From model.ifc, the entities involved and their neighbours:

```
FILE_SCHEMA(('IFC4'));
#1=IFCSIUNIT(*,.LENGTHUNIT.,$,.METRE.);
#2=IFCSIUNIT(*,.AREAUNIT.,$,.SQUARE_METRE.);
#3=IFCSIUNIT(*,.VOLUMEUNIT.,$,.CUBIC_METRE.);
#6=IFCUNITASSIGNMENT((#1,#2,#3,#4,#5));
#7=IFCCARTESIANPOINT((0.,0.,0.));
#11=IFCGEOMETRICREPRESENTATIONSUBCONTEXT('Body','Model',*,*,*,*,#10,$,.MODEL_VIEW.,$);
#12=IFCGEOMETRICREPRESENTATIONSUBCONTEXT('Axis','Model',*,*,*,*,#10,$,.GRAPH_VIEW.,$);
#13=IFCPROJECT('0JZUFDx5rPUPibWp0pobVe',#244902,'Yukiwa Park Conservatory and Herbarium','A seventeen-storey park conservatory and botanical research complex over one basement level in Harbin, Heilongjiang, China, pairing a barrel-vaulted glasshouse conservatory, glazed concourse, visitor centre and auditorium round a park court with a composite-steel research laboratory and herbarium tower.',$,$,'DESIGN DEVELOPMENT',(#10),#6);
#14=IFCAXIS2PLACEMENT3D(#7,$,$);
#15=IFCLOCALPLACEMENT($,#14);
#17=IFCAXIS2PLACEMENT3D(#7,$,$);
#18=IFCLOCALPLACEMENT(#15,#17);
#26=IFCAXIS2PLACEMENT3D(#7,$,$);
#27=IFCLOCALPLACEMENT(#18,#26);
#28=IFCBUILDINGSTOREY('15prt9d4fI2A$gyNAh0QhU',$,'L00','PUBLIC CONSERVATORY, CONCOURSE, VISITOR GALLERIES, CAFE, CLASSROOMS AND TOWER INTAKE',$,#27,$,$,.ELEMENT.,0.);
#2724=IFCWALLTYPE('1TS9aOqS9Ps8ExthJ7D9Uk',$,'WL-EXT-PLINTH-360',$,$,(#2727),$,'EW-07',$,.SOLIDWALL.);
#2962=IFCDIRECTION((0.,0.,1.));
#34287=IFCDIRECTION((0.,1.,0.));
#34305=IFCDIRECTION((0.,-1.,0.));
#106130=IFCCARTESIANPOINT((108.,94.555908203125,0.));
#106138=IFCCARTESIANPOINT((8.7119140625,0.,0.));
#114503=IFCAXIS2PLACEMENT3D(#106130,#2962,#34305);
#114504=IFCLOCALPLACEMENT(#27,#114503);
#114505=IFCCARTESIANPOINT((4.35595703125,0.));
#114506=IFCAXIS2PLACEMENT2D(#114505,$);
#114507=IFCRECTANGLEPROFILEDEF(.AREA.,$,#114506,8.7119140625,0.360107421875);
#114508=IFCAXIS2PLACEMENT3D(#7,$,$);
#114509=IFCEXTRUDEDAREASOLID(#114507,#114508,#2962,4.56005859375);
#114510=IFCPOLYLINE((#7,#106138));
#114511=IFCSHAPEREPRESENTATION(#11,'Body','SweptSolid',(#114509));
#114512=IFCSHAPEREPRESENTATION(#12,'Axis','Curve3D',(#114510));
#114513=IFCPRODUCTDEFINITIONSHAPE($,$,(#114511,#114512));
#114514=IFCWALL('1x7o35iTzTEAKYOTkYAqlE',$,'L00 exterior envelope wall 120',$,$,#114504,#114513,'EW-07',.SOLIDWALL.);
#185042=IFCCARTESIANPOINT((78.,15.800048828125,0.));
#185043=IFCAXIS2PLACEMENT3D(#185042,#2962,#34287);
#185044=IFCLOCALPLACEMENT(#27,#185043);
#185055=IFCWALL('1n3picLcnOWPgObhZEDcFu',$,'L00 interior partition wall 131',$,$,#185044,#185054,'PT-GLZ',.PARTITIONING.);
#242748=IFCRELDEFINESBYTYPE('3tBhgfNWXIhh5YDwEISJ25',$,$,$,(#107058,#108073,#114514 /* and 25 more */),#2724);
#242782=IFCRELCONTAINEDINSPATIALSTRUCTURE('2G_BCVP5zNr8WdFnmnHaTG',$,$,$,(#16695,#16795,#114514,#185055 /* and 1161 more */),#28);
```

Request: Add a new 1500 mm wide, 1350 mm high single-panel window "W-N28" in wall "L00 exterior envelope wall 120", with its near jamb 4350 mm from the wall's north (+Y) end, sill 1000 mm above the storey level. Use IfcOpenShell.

```python
import numpy as np
import ifcopenshell
import ifcopenshell.api.feature
import ifcopenshell.api.geometry
import ifcopenshell.api.root
import ifcopenshell.api.spatial
import ifcopenshell.geom
import ifcopenshell.util.element
import ifcopenshell.util.placement
import ifcopenshell.util.representation
import ifcopenshell.util.shape
import ifcopenshell.util.unit

model = ifcopenshell.open("model.ifc")
unit_scale = ifcopenshell.util.unit.calculate_unit_scale(model)
settings = ifcopenshell.geom.settings()


def volume(element):
    """Net volume in cubic metres, openings subtracted."""
    shape = ifcopenshell.geom.create_shape(settings, element)
    return ifcopenshell.util.shape.get_volume(shape.geometry)


wall = model.by_guid("1x7o35iTzTEAKYOTkYAqlE")
storey = ifcopenshell.util.element.get_container(wall, ifc_class="IfcBuildingStorey")
context = ifcopenshell.util.representation.get_context(model, "Model", "Body", "MODEL_VIEW")
before = volume(wall)

width, height, from_end, sill = 1.5, 1.35, 4.35, 1  # metres

# The wall runs along its own X axis, and the end named is its -X end.
wall_shape = ifcopenshell.geom.create_shape(settings, wall)
x, y, z = ifcopenshell.util.shape.get_vertices(wall_shape.geometry).T
start = x.min() + from_end
face, thickness = float(y.min()), float(y.max() - y.min())
wall_matrix = ifcopenshell.util.placement.get_local_placement(wall.ObjectPlacement)
level = ifcopenshell.util.placement.get_local_placement(storey.ObjectPlacement)[2, 3]


def in_wall(x, y):
    """Placement at x, y metres in the wall's axes, at sill height."""
    matrix = wall_matrix.copy()
    matrix[:, 3] = wall_matrix @ np.array([x / unit_scale, y / unit_scale, 0.0, 1.0])
    matrix[2, 3] = level + sill / unit_scale
    return matrix


# Opening: a box that overshoots both wall faces by 50 mm.
opening = ifcopenshell.api.root.create_entity(model, ifc_class="IfcOpeningElement", predefined_type="OPENING")
box = ifcopenshell.api.geometry.add_wall_representation(
    model, context=context, length=width, height=height, thickness=thickness + 0.1
)
ifcopenshell.api.geometry.assign_representation(model, product=opening, representation=box)
ifcopenshell.api.geometry.edit_object_placement(model, product=opening, matrix=in_wall(start, face - 0.05), is_si=False)
ifcopenshell.api.feature.add_feature(model, feature=opening, element=wall)

window = ifcopenshell.api.root.create_entity(model, ifc_class="IfcWindow", name="W-N28", predefined_type="WINDOW")
window.OverallWidth, window.OverallHeight = width / unit_scale, height / unit_scale
window.PartitioningType = "SINGLE_PANEL"
body = ifcopenshell.api.geometry.add_window_representation(
    model,
    context=context,
    overall_width=window.OverallWidth,
    overall_height=window.OverallHeight,
    partition_type="SINGLE_PANEL",
)
ifcopenshell.api.geometry.assign_representation(model, product=window, representation=body)
ifcopenshell.api.spatial.assign_container(model, products=[window], relating_structure=storey)
ifcopenshell.api.feature.add_filling(model, opening=opening, element=window)

# Centre the window in the wall's thickness.
ifcopenshell.api.geometry.edit_object_placement(model, product=window, matrix=in_wall(start, face), is_si=False)
window_shape = ifcopenshell.geom.create_shape(settings, window)
depth = ifcopenshell.util.shape.get_vertices(window_shape.geometry)[:, 1]
offset = face + thickness / 2 - (depth.min() + depth.max()) / 2
ifcopenshell.api.geometry.edit_object_placement(model, product=window, matrix=in_wall(start, offset), is_si=False)

after = volume(wall)

print(f"wall volume {before:.3f} -> {after:.3f} m3")

model.write("model_edited.ifc")
```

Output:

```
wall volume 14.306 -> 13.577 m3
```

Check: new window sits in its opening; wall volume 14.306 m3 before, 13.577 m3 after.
